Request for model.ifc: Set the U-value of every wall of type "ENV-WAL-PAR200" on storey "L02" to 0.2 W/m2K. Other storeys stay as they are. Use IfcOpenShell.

First a look at what the model holds.

```python
import ifcopenshell
import ifcopenshell.util.element

model = ifcopenshell.open("model.ifc")
print(model.schema)
storey = next(s for s in model.by_type("IfcBuildingStorey") if s.Name == "L02")
walls = [e for e in ifcopenshell.util.element.get_decomposition(storey) if e.is_a("IfcWall")]
seen = {}
for e in walls:
    element_type = ifcopenshell.util.element.get_type(e)
    key = (element_type.Name if element_type != e and element_type else None, ifcopenshell.util.element.get_pset(e, "Pset_WallCommon", "ThermalTransmittance"))
    seen[key] = seen.get(key, 0) + 1
for (name, value), count in sorted(seen.items(), key=str):
    print(count, "x", name, "|", value)
```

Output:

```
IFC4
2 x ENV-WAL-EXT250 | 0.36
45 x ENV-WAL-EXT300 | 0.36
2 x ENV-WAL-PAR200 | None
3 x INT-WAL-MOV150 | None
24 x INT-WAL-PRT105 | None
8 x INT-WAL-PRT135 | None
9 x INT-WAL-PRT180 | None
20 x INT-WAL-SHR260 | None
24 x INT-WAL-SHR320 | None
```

```python
import ifcopenshell
import ifcopenshell.api.pset
import ifcopenshell.util.element

model = ifcopenshell.open("model.ifc")

storey = next(s for s in model.by_type("IfcBuildingStorey") if s.Name == "L02")
walls = [e for e in ifcopenshell.util.element.get_decomposition(storey) if e.is_a("IfcWall")]

count = 0
for e in walls:
    element_type = ifcopenshell.util.element.get_type(e)
    if element_type in (None, e) or element_type.Name != "ENV-WAL-PAR200":
        continue
    # add_pset returns the element's existing set when there is one.
    pset = ifcopenshell.api.pset.add_pset(model, product=e, name="Pset_WallCommon")
    ifcopenshell.api.pset.edit_pset(model, pset=pset, properties={"ThermalTransmittance": 0.2})
    count += 1

print(count, "walls updated")

model.write("model_edited.ifc")
```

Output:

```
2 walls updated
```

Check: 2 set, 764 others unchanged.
